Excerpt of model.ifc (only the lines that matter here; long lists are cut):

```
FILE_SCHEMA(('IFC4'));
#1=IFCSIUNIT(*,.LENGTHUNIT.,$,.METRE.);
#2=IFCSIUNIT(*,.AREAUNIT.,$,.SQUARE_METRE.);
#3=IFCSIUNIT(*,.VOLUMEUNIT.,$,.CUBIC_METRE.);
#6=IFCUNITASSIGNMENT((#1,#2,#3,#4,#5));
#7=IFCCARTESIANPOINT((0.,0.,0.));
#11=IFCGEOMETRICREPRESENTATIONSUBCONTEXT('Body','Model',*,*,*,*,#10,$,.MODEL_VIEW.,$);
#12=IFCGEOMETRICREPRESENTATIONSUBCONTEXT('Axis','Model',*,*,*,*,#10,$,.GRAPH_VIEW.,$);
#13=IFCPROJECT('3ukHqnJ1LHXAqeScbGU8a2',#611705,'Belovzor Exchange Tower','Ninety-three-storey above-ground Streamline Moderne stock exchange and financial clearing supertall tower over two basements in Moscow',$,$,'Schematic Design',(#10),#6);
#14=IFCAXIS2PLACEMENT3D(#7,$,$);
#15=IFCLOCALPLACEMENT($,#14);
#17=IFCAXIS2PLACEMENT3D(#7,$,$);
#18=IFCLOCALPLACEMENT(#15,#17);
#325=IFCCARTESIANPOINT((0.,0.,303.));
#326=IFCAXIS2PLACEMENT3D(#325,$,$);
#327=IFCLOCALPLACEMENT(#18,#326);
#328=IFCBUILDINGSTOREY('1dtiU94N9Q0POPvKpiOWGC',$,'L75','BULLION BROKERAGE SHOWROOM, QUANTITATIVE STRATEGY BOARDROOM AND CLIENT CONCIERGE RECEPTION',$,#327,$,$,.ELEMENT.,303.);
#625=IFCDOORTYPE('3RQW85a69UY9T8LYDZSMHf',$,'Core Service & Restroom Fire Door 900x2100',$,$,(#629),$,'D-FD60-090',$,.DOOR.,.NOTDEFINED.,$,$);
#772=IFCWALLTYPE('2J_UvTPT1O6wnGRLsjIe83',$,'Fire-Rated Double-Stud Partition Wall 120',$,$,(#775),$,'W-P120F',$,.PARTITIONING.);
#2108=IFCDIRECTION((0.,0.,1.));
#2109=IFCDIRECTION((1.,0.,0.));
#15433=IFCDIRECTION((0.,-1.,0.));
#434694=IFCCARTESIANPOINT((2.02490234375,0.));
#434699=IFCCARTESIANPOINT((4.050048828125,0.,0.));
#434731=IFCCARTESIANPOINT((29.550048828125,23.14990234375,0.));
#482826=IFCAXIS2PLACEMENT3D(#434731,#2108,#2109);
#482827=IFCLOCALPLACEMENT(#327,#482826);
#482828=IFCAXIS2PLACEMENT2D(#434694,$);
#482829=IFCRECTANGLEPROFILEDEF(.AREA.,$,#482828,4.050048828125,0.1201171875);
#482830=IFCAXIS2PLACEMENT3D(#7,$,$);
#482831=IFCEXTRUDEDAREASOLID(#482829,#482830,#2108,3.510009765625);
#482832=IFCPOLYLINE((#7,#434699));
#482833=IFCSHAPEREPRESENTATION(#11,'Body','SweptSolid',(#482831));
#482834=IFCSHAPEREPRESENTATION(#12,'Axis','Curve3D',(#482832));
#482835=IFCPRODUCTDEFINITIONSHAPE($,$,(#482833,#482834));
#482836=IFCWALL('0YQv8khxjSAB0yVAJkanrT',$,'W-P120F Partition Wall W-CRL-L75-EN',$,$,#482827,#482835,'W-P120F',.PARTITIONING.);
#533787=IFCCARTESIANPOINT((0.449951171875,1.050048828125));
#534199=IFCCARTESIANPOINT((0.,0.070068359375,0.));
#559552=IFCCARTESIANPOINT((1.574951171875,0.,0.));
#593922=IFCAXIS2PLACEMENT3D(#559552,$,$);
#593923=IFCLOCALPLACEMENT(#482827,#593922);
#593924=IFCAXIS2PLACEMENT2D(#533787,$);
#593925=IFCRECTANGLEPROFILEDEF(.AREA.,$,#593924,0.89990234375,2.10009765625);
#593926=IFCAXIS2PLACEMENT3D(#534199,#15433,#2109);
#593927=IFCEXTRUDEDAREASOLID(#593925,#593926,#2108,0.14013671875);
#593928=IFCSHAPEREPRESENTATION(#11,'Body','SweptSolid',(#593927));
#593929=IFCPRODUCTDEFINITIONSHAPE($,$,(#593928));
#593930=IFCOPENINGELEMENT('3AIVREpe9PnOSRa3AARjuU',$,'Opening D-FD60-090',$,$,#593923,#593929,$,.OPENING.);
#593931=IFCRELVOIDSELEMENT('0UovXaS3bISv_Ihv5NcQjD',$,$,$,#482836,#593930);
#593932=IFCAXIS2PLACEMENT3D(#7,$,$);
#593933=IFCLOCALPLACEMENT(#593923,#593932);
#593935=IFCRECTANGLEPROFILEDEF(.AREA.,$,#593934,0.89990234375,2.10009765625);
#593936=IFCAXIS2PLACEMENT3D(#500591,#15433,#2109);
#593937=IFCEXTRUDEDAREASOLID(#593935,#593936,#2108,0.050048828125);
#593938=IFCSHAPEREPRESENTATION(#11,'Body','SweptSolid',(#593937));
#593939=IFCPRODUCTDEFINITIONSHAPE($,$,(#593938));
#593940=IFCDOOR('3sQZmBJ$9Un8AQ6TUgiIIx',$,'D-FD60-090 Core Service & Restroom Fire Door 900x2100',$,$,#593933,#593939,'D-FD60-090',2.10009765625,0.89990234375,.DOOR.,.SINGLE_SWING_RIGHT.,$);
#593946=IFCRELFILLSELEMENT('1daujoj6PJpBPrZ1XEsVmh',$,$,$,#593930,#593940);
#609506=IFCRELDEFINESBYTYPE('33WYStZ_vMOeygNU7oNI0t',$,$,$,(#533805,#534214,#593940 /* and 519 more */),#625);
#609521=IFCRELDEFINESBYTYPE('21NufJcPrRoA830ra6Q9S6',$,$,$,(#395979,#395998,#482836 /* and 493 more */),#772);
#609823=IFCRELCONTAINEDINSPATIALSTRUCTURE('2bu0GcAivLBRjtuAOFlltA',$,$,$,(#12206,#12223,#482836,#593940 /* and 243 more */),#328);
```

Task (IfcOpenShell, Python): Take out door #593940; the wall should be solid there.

```python
import ifcopenshell
import ifcopenshell.api.feature
import ifcopenshell.api.root
import ifcopenshell.geom
import ifcopenshell.util.shape

model = ifcopenshell.open("model.ifc")
settings = ifcopenshell.geom.settings()


def volume(element):
    """Net volume in cubic metres, openings subtracted."""
    shape = ifcopenshell.geom.create_shape(settings, element)
    return ifcopenshell.util.shape.get_volume(shape.geometry)


door = model.by_guid("3sQZmBJ$9Un8AQ6TUgiIIx")
opening = door.FillsVoids[0].RelatingOpeningElement
wall = opening.VoidsElements[0].RelatingBuildingElement
before = volume(wall)

ifcopenshell.api.root.remove_product(model, product=door)
ifcopenshell.api.feature.remove_feature(model, feature=opening)

after = volume(wall)

print(f"wall volume {before:.3f} -> {after:.3f} m3")

model.write("model_v2.ifc")
```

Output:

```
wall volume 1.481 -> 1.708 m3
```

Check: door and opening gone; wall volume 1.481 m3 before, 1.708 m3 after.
